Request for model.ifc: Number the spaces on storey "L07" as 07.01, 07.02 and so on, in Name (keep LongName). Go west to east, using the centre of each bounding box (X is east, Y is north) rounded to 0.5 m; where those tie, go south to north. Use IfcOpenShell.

First a look at what the model holds.

```python
import ifcopenshell
import ifcopenshell.util.element
import ifcopenshell.util.placement

model = ifcopenshell.open("model.ifc")
print(model.schema)
storey = next(s for s in model.by_type("IfcBuildingStorey") if s.Name == "L07")
spaces = [e for e in ifcopenshell.util.element.get_decomposition(storey) if e.is_a("IfcSpace")]
for e in sorted(spaces, key=lambda e: e.id()):
    origin = ifcopenshell.util.placement.get_local_placement(e.ObjectPlacement)[:3, 3]
    print(e.id(), e.Name, e.LongName, origin.round(2) + 0.0, sep=" | ")
```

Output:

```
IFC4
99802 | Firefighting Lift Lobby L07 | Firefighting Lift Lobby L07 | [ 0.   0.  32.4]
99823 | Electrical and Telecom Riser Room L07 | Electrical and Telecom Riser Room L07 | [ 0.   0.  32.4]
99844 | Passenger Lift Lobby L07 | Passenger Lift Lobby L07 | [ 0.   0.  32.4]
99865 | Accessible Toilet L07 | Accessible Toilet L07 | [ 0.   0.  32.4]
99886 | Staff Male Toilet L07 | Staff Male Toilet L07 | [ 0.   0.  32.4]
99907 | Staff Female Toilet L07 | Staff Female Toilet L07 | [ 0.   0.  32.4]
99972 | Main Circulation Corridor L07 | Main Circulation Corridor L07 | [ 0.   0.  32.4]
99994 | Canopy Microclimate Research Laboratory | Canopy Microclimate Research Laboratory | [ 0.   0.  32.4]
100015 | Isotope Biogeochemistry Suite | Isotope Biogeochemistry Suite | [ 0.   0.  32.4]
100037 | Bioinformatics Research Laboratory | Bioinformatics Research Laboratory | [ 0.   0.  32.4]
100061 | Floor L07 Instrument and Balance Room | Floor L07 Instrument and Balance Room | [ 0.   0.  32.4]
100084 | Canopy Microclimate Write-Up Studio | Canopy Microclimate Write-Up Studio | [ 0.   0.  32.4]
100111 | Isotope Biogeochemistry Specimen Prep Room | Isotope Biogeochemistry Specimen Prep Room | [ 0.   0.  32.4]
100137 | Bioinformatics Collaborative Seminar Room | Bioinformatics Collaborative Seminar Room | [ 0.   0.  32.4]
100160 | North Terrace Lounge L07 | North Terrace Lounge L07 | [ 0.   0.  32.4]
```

```python
import ifcopenshell
import ifcopenshell.geom
import ifcopenshell.util.element
import ifcopenshell.util.shape

model = ifcopenshell.open("model.ifc")
settings = ifcopenshell.geom.settings()
settings.set("use-world-coords", True)


def centre(element):
    shape = ifcopenshell.geom.create_shape(settings, element)
    return ifcopenshell.util.shape.get_bbox_centroid(shape.geometry)


storey = next(s for s in model.by_type("IfcBuildingStorey") if s.Name == "L07")
spaces = [e for e in ifcopenshell.util.element.get_decomposition(storey) if e.is_a("IfcSpace")]

# Insertion points can sit at a corner or the storey origin, so sort by the geometry (in metres).
centres = {e: centre(e) for e in spaces}
spaces.sort(key=lambda e: (round(centres[e][0] / 0.5), centres[e][1]))

for i, e in enumerate(spaces, start=1):
    number = f"07.{i:02d}"
    e.Name = number
    print(e.id(), number)

model.write("model_v2.ifc")
```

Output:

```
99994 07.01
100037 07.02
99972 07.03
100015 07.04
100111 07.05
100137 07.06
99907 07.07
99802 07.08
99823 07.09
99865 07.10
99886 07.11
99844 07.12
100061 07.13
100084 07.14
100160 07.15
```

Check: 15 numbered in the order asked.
